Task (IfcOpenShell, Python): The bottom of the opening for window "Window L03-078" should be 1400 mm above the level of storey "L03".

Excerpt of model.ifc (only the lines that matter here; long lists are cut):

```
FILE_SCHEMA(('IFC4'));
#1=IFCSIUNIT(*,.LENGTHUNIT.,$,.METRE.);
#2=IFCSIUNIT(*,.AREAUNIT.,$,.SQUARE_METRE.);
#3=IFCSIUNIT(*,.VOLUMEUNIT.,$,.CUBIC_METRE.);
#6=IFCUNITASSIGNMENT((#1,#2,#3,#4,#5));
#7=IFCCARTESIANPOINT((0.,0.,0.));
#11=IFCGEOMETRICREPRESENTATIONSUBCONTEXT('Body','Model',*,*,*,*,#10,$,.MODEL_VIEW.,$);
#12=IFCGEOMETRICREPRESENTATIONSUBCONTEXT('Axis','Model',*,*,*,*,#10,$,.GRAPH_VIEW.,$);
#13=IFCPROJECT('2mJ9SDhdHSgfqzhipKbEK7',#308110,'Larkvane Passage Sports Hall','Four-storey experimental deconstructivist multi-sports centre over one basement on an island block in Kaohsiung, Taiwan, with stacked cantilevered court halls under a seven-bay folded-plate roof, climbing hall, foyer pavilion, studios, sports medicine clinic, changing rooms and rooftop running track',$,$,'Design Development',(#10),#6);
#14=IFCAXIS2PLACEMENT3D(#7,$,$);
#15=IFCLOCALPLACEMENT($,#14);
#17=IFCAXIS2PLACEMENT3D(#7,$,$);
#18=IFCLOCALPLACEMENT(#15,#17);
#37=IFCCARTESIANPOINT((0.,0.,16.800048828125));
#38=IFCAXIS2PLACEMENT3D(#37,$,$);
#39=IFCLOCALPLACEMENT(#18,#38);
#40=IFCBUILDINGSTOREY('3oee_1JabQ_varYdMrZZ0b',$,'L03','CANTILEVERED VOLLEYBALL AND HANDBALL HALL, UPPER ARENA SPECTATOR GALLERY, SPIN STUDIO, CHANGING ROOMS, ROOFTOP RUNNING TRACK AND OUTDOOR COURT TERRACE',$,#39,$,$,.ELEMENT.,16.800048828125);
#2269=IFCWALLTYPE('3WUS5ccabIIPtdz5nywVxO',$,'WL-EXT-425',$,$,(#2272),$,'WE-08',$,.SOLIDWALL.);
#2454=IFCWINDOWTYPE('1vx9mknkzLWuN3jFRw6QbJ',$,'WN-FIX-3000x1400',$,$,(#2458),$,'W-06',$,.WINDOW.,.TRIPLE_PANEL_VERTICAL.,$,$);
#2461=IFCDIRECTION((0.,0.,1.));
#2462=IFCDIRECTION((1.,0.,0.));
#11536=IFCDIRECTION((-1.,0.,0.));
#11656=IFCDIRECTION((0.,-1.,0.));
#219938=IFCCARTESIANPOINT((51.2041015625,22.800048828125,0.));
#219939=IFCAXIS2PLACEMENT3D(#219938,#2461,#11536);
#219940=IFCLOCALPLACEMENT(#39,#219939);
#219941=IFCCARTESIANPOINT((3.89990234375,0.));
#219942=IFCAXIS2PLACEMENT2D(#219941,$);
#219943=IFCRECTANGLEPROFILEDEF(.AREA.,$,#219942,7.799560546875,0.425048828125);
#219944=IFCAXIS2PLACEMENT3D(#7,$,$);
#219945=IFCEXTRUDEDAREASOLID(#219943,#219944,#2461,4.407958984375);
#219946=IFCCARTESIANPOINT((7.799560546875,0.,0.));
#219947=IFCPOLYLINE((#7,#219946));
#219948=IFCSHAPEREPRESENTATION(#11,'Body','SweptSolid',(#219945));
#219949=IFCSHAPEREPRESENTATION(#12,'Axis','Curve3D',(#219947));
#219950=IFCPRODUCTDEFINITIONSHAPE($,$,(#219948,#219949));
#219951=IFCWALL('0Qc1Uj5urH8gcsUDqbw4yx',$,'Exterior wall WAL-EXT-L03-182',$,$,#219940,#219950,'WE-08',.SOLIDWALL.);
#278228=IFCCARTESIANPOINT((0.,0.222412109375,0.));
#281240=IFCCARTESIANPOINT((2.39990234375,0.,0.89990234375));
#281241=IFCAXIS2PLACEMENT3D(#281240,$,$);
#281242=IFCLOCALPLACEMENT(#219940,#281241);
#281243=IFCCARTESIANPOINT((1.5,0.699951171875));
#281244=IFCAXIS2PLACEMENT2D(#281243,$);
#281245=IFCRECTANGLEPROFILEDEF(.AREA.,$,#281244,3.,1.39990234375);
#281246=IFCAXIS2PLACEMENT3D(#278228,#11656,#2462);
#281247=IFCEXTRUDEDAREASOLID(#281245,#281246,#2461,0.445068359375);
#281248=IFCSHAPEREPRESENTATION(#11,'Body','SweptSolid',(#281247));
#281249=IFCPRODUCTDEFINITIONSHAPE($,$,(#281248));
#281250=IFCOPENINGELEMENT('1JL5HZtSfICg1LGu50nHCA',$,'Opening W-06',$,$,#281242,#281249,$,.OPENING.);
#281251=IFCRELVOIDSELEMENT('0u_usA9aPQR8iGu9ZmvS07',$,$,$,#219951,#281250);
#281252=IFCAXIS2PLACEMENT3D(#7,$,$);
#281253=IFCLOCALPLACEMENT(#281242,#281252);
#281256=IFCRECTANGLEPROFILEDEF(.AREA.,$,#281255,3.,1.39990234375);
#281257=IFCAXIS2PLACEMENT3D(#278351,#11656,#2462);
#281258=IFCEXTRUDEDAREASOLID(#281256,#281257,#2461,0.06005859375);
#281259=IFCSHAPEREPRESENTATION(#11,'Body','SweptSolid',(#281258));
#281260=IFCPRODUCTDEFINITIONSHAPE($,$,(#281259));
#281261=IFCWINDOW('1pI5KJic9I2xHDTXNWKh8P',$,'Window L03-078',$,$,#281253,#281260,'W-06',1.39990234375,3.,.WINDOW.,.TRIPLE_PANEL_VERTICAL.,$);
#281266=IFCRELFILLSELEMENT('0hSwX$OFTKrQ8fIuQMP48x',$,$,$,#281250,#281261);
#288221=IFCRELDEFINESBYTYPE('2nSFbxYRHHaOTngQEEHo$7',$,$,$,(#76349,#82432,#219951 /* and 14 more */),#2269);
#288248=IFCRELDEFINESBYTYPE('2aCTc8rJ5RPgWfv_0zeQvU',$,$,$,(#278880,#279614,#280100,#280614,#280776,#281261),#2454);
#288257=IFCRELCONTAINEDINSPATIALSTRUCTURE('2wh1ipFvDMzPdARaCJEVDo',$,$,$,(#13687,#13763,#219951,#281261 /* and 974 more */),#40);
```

```python
import numpy as np
import ifcopenshell
import ifcopenshell.api.geometry
import ifcopenshell.geom
import ifcopenshell.util.element
import ifcopenshell.util.placement
import ifcopenshell.util.shape
import ifcopenshell.util.unit

model = ifcopenshell.open("model.ifc")
unit_scale = ifcopenshell.util.unit.calculate_unit_scale(model)

window = model.by_id(281261)
opening = window.FillsVoids[0].RelatingOpeningElement
storey = ifcopenshell.util.element.get_container(window, ifc_class="IfcBuildingStorey")
level = ifcopenshell.util.placement.get_local_placement(storey.ObjectPlacement)[2, 3]

# The opening's origin need not be at the sill, so measure its lowest point.
shape = ifcopenshell.geom.create_shape(ifcopenshell.geom.settings(), opening)
bottom = ifcopenshell.util.shape.get_shape_bottom_elevation(shape, shape.geometry) / unit_scale
dz = level + 1.4 / unit_scale - bottom

shift = np.array([0.0, 0.0, dz])
# The window is placed relative to its opening, so it follows when the opening moves.
matrix = ifcopenshell.util.placement.get_local_placement(opening.ObjectPlacement)
matrix[:3, 3] += shift
ifcopenshell.api.geometry.edit_object_placement(
    model, product=opening, matrix=matrix, is_si=False, should_transform_children=True
)

print(f"moved by {dz * unit_scale:+.3f} m")

model.write("model_edited.ifc")
```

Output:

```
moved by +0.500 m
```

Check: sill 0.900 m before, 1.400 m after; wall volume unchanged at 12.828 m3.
